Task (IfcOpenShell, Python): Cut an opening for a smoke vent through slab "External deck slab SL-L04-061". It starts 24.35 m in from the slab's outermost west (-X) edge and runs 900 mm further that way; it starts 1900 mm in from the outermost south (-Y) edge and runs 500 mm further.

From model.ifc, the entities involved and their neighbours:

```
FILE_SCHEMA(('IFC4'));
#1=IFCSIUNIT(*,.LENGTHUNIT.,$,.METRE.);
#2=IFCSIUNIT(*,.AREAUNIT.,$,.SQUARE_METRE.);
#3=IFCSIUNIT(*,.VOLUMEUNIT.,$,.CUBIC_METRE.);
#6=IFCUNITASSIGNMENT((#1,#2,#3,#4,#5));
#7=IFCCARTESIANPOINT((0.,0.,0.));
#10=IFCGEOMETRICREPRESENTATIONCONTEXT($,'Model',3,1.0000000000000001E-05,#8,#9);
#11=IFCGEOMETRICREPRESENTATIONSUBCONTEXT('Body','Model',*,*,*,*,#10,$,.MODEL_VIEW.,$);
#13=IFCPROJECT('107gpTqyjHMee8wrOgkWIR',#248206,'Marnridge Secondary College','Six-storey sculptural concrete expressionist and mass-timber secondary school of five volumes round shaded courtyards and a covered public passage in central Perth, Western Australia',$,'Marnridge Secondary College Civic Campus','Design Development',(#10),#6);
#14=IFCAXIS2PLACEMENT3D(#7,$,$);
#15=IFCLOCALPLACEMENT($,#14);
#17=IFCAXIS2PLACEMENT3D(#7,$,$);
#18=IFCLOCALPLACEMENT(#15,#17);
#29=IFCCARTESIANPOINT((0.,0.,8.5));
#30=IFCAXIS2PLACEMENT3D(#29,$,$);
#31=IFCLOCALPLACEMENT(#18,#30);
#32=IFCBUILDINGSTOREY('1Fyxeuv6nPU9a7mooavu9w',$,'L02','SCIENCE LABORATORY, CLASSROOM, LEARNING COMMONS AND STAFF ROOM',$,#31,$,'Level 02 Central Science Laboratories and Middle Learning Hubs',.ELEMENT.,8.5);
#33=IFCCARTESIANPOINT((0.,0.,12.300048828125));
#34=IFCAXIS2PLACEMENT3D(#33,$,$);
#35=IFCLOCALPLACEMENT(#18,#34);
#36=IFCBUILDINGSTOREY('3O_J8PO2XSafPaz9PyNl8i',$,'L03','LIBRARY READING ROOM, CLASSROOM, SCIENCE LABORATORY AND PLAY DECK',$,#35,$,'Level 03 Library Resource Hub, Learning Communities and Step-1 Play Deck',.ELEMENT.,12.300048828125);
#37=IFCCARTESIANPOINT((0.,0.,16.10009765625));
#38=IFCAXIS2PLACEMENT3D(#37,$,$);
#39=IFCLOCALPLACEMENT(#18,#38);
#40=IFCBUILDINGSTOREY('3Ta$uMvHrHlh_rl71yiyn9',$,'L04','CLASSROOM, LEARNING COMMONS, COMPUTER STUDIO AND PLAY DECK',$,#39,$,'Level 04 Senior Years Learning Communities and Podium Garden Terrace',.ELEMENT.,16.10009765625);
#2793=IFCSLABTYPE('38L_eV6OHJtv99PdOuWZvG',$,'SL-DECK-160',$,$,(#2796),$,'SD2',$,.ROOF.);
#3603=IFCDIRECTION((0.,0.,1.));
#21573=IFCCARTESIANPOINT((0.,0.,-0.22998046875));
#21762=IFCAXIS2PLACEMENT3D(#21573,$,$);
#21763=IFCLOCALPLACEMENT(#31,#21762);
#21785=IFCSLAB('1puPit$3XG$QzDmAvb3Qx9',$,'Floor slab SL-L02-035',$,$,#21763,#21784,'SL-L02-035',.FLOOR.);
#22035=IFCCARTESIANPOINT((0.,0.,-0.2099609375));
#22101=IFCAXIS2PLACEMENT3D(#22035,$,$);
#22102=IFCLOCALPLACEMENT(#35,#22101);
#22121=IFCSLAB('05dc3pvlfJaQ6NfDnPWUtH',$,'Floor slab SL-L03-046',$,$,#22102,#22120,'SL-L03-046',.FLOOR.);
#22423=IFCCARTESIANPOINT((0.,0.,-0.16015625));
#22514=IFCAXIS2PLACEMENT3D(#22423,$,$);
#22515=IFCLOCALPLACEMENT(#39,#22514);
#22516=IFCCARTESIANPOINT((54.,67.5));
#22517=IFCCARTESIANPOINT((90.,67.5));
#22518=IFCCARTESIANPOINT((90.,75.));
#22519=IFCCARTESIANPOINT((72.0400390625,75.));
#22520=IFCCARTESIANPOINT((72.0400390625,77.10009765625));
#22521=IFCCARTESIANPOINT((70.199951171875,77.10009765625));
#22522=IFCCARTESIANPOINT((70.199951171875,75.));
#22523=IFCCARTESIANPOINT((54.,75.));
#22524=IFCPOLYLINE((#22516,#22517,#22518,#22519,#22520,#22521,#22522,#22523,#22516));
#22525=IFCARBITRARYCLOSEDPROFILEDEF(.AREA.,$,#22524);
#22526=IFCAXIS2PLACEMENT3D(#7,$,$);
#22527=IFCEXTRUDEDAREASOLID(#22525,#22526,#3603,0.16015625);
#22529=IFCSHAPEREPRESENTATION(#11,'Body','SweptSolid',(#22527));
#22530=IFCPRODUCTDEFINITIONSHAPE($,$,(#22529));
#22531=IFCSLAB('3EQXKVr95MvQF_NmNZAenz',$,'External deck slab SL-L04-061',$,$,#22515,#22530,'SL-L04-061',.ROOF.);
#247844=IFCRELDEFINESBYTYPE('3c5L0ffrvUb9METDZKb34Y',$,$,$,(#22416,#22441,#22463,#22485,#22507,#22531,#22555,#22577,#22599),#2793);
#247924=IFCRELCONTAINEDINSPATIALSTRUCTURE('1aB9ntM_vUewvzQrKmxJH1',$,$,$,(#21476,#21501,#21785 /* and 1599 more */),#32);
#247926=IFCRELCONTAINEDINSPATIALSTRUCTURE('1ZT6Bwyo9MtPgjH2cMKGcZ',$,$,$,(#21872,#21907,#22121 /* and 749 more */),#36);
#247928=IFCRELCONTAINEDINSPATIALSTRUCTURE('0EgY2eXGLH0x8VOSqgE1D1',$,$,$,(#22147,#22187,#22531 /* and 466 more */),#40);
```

```python
import numpy as np
import ifcopenshell
import ifcopenshell.api.feature
import ifcopenshell.api.geometry
import ifcopenshell.api.root
import ifcopenshell.geom
import ifcopenshell.util.placement
import ifcopenshell.util.representation
import ifcopenshell.util.shape
import ifcopenshell.util.unit

model = ifcopenshell.open("model.ifc")
unit_scale = ifcopenshell.util.unit.calculate_unit_scale(model)
settings = ifcopenshell.geom.settings()


def volume(element):
    """Net volume in cubic metres, openings subtracted."""
    shape = ifcopenshell.geom.create_shape(settings, element)
    return ifcopenshell.util.shape.get_volume(shape.geometry)


slab = model.by_guid("3EQXKVr95MvQF_NmNZAenz")
before = volume(slab)

# Extent in the slab's own axes, in metres. The edges named are its -X and -Y sides.
slab_shape = ifcopenshell.geom.create_shape(settings, slab)
vertices = ifcopenshell.util.shape.get_vertices(slab_shape.geometry)
x_min, y_min, bottom = vertices.min(axis=0)
top = vertices[:, 2].max()

opening = ifcopenshell.api.root.create_entity(model, ifc_class="IfcOpeningElement", name="Smoke vent opening", predefined_type="OPENING")
context = ifcopenshell.util.representation.get_context(model, "Model", "Body", "MODEL_VIEW")
width, depth = 0.9, 0.5
outline = [(0.0, 0.0), (width, 0.0), (width, depth), (0.0, depth), (0.0, 0.0)]
# Overshoot both faces by 50 mm so the cut is clean.
shape = ifcopenshell.api.geometry.add_slab_representation(
    model, context=context, depth=top - bottom + 0.1, polyline=outline
)
ifcopenshell.api.geometry.assign_representation(model, product=opening, representation=shape)

matrix = ifcopenshell.util.placement.get_local_placement(slab.ObjectPlacement)
matrix[:, 3] = matrix @ np.append(np.array([x_min + 24.35, y_min + 1.9, bottom - 0.05]) / unit_scale, 1.0)
ifcopenshell.api.geometry.edit_object_placement(model, product=opening, matrix=matrix, is_si=False)
ifcopenshell.api.feature.add_feature(model, feature=opening, element=slab)

after = volume(slab)

print(f"slab volume {before:.3f} -> {after:.3f} m3")

model.write("model_edited.ifc")
```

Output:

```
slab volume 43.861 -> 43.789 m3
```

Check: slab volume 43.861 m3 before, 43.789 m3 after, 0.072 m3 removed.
